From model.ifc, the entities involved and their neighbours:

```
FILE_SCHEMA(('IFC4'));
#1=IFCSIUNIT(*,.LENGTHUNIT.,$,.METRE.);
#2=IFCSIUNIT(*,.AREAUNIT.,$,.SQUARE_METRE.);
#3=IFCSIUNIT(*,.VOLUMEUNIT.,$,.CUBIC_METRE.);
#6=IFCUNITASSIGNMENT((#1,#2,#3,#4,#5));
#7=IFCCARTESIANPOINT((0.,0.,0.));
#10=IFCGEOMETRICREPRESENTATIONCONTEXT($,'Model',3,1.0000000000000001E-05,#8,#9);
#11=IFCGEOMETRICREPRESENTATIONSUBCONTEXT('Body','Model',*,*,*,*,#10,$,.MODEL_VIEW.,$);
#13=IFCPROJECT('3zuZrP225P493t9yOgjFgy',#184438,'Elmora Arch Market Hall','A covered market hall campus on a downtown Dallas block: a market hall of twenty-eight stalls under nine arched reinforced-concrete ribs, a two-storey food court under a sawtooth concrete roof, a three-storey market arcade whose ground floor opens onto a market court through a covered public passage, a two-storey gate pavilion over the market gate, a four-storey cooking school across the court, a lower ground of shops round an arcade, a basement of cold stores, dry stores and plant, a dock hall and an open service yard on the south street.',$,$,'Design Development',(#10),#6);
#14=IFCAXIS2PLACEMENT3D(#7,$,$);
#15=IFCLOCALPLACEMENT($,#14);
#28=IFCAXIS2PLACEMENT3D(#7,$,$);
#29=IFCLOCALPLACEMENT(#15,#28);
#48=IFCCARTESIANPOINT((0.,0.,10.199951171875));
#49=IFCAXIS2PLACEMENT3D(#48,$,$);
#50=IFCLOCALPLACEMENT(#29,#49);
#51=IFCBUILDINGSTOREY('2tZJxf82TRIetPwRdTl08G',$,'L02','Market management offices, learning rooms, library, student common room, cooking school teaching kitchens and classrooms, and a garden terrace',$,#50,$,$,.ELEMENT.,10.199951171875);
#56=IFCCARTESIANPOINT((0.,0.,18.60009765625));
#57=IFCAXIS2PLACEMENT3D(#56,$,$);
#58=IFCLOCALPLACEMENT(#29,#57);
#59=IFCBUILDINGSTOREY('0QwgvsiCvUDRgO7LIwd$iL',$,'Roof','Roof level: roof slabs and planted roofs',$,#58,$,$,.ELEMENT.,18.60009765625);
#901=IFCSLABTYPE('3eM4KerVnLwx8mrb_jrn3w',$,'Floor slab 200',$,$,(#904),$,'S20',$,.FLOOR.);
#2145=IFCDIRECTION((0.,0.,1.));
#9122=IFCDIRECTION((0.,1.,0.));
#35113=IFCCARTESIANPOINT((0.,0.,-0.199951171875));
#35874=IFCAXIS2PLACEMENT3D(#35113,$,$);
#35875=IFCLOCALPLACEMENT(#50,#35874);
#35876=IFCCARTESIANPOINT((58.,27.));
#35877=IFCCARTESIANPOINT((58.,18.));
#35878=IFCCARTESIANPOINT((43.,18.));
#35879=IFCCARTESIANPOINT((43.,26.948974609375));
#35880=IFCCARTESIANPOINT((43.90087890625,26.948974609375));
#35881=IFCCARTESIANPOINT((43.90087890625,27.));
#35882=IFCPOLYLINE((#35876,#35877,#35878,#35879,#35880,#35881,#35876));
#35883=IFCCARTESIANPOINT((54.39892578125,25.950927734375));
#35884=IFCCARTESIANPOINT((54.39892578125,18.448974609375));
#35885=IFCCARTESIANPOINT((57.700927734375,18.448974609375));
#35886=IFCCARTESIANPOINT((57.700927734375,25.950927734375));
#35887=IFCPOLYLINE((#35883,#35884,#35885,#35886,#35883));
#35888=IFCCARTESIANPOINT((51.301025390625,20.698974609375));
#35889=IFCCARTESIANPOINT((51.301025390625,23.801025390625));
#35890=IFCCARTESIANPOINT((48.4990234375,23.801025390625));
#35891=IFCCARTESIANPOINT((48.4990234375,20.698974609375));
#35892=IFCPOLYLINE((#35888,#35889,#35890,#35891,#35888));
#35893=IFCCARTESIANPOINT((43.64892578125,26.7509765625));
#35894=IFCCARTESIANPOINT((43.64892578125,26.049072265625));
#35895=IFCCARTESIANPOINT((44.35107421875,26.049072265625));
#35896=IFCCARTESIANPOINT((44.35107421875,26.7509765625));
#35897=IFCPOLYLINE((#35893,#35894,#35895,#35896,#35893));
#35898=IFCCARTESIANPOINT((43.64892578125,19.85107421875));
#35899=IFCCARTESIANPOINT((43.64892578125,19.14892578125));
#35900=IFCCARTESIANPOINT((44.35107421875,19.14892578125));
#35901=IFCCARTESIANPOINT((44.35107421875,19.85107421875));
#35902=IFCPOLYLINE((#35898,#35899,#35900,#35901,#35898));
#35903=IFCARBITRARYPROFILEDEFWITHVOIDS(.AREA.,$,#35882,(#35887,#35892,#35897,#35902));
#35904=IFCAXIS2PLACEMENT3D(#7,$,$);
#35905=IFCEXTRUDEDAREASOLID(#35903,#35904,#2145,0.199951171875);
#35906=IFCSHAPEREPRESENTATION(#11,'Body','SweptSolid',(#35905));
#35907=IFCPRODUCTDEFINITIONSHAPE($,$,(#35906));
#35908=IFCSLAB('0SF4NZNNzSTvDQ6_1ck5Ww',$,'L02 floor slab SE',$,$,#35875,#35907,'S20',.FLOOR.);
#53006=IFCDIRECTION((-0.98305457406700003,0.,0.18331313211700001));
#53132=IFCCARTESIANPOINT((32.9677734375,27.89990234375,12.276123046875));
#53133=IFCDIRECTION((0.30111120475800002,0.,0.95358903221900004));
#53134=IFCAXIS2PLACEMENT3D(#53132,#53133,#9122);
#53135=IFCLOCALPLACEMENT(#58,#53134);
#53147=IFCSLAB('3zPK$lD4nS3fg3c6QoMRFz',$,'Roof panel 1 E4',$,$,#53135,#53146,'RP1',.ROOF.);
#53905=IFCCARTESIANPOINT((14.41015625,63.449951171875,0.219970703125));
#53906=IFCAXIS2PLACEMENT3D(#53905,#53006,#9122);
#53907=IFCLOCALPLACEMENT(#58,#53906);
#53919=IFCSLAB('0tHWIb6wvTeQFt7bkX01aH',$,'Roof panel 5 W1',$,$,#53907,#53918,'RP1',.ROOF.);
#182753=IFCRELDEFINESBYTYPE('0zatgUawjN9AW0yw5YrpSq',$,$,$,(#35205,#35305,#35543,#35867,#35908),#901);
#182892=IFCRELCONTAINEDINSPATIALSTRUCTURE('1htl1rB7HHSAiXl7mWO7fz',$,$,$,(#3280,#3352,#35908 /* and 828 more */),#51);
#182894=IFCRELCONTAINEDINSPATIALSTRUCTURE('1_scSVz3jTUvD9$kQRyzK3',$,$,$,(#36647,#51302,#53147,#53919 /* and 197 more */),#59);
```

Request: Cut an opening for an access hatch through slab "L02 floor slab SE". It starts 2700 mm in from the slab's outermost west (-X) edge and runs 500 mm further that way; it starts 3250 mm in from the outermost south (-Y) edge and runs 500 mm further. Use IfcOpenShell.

```python
import numpy as np
import ifcopenshell
import ifcopenshell.api.feature
import ifcopenshell.api.geometry
import ifcopenshell.api.root
import ifcopenshell.geom
import ifcopenshell.util.placement
import ifcopenshell.util.representation
import ifcopenshell.util.shape
import ifcopenshell.util.unit

model = ifcopenshell.open("model.ifc")
unit_scale = ifcopenshell.util.unit.calculate_unit_scale(model)
settings = ifcopenshell.geom.settings()


def volume(element):
    """Net volume in cubic metres, openings subtracted."""
    shape = ifcopenshell.geom.create_shape(settings, element)
    return ifcopenshell.util.shape.get_volume(shape.geometry)


slab = model.by_guid("0SF4NZNNzSTvDQ6_1ck5Ww")
before = volume(slab)

# Extent in the slab's own axes, in metres. The edges named are its -X and -Y sides.
slab_shape = ifcopenshell.geom.create_shape(settings, slab)
vertices = ifcopenshell.util.shape.get_vertices(slab_shape.geometry)
x_min, y_min, bottom = vertices.min(axis=0)
top = vertices[:, 2].max()

opening = ifcopenshell.api.root.create_entity(model, ifc_class="IfcOpeningElement", name="Access hatch opening", predefined_type="OPENING")
context = ifcopenshell.util.representation.get_context(model, "Model", "Body", "MODEL_VIEW")
width, depth = 0.5, 0.5
outline = [(0.0, 0.0), (width, 0.0), (width, depth), (0.0, depth), (0.0, 0.0)]
# Overshoot both faces by 50 mm so the cut is clean.
shape = ifcopenshell.api.geometry.add_slab_representation(
    model, context=context, depth=top - bottom + 0.1, polyline=outline
)
ifcopenshell.api.geometry.assign_representation(model, product=opening, representation=shape)

matrix = ifcopenshell.util.placement.get_local_placement(slab.ObjectPlacement)
matrix[:, 3] = matrix @ np.append(np.array([x_min + 2.7, y_min + 3.25, bottom - 0.05]) / unit_scale, 1.0)
ifcopenshell.api.geometry.edit_object_placement(model, product=opening, matrix=matrix, is_si=False)
ifcopenshell.api.feature.add_feature(model, feature=opening, element=slab)

after = volume(slab)

print(f"slab volume {before:.3f} -> {after:.3f} m3")

model.write("model_rev.ifc")
```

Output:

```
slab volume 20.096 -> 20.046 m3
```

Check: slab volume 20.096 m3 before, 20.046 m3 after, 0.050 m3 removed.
